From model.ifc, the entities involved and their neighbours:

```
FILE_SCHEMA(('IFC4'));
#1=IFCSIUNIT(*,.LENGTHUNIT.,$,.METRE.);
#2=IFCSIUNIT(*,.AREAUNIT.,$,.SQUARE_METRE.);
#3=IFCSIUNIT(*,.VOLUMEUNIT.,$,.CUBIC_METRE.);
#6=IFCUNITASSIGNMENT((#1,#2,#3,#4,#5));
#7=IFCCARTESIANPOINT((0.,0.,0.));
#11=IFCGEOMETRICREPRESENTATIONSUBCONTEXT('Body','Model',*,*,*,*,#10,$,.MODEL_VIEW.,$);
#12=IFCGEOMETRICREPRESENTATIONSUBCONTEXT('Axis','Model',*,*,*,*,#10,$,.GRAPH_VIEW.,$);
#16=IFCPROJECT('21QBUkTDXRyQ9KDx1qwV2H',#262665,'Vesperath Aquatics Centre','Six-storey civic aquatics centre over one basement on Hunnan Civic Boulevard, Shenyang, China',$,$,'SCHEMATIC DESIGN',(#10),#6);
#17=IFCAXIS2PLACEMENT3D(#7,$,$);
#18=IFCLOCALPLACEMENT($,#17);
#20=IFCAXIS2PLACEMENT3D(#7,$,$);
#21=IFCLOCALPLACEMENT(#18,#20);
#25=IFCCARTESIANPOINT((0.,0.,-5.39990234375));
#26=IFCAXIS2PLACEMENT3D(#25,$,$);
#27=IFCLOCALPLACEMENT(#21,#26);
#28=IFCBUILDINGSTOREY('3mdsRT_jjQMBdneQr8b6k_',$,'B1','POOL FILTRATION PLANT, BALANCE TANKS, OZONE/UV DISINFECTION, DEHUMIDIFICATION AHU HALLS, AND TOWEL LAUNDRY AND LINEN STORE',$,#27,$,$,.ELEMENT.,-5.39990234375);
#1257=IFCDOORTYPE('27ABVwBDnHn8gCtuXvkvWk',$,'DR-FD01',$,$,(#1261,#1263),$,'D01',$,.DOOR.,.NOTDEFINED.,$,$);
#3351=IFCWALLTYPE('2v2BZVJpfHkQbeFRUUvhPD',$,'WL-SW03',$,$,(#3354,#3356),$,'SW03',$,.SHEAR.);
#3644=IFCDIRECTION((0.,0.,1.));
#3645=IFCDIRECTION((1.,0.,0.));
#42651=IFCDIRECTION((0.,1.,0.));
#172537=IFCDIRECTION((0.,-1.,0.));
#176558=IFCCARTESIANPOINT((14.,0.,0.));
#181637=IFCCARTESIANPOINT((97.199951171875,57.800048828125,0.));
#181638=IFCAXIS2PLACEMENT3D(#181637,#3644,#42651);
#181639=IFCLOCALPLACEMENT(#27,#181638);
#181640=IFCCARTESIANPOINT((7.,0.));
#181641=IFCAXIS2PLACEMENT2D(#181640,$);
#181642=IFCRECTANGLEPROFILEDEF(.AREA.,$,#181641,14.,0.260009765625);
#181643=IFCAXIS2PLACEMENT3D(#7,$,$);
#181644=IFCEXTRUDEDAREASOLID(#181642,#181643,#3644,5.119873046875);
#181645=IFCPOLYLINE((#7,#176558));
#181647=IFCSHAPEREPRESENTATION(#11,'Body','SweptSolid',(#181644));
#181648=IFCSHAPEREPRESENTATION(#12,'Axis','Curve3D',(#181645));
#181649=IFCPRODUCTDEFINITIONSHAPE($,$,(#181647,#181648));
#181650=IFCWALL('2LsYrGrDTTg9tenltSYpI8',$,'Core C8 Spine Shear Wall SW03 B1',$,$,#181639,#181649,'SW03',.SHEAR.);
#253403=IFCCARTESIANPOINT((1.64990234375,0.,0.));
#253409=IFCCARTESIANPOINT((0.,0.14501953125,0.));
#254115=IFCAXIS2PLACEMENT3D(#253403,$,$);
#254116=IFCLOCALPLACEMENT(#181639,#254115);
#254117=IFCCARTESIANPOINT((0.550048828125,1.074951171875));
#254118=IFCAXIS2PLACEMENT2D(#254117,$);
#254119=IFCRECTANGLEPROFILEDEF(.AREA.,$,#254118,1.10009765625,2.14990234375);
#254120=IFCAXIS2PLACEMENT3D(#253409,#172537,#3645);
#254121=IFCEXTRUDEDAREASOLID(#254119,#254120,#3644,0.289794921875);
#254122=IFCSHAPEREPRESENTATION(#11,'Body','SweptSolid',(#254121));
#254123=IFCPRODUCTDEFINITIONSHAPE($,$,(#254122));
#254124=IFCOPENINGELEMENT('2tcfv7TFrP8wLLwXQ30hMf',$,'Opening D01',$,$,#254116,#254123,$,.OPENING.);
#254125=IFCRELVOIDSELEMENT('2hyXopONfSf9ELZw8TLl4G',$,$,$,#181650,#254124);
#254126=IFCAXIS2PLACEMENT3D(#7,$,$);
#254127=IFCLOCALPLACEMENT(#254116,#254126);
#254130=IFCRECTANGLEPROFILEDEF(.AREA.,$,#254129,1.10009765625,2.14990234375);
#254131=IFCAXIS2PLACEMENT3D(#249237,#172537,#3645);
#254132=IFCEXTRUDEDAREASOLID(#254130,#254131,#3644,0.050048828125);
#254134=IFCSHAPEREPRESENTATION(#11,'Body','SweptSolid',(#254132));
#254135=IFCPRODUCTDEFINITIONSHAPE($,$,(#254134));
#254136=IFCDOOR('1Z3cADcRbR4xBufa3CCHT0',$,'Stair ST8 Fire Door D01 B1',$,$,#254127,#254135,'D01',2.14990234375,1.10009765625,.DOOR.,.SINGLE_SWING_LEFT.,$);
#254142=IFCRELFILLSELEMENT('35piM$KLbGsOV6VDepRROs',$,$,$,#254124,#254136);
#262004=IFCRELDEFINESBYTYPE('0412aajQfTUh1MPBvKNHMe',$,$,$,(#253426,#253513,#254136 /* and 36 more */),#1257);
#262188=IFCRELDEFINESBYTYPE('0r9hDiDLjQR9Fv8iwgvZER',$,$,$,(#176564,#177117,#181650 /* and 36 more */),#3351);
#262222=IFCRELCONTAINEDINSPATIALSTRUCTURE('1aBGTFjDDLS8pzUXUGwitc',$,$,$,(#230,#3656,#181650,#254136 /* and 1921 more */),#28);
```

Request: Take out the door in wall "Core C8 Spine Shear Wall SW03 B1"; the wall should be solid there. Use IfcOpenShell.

```python
import ifcopenshell
import ifcopenshell.api.feature
import ifcopenshell.api.root
import ifcopenshell.geom
import ifcopenshell.util.shape

model = ifcopenshell.open("model.ifc")
settings = ifcopenshell.geom.settings()


def volume(element):
    """Net volume in cubic metres, openings subtracted."""
    shape = ifcopenshell.geom.create_shape(settings, element)
    return ifcopenshell.util.shape.get_volume(shape.geometry)


door = model.by_guid("1Z3cADcRbR4xBufa3CCHT0")
opening = door.FillsVoids[0].RelatingOpeningElement
wall = opening.VoidsElements[0].RelatingBuildingElement
before = volume(wall)

ifcopenshell.api.root.remove_product(model, product=door)
ifcopenshell.api.feature.remove_feature(model, feature=opening)

after = volume(wall)

print(f"wall volume {before:.3f} -> {after:.3f} m3")

model.write("model_edited.ifc")
```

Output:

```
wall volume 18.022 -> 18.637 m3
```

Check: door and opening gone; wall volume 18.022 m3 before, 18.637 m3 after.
